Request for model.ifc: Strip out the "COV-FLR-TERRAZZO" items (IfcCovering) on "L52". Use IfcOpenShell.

First a look at what the model holds.

```python
import ifcopenshell
import ifcopenshell.util.element

model = ifcopenshell.open("model.ifc")
print(model.schema)
storey = next(s for s in model.by_type("IfcBuildingStorey") if s.Name == "L52")
coverings = [e for e in ifcopenshell.util.element.get_decomposition(storey) if e.is_a("IfcCovering")]
seen = {}
for e in coverings:
    element_type = ifcopenshell.util.element.get_type(e)
    name = element_type.Name if element_type not in (None, e) else None
    seen[name] = seen.get(name, 0) + 1
for name, count in sorted(seen.items(), key=str):
    print(count, "x", name)
```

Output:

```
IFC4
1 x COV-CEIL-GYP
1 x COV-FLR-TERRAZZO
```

```python
import ifcopenshell
import ifcopenshell.api.root
import ifcopenshell.util.element

model = ifcopenshell.open("model.ifc")

storey = next(s for s in model.by_type("IfcBuildingStorey") if s.Name == "L52")
coverings = [e for e in ifcopenshell.util.element.get_decomposition(storey) if e.is_a("IfcCovering")]
targets = [e for e in coverings if (t := ifcopenshell.util.element.get_type(e)) not in (None, e) and t.Name == "COV-FLR-TERRAZZO"]

for e in targets:
    ifcopenshell.api.root.remove_product(model, product=e)
print(len(targets), "removed")

model.write("model_rev.ifc")
```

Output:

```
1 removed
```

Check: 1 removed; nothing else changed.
